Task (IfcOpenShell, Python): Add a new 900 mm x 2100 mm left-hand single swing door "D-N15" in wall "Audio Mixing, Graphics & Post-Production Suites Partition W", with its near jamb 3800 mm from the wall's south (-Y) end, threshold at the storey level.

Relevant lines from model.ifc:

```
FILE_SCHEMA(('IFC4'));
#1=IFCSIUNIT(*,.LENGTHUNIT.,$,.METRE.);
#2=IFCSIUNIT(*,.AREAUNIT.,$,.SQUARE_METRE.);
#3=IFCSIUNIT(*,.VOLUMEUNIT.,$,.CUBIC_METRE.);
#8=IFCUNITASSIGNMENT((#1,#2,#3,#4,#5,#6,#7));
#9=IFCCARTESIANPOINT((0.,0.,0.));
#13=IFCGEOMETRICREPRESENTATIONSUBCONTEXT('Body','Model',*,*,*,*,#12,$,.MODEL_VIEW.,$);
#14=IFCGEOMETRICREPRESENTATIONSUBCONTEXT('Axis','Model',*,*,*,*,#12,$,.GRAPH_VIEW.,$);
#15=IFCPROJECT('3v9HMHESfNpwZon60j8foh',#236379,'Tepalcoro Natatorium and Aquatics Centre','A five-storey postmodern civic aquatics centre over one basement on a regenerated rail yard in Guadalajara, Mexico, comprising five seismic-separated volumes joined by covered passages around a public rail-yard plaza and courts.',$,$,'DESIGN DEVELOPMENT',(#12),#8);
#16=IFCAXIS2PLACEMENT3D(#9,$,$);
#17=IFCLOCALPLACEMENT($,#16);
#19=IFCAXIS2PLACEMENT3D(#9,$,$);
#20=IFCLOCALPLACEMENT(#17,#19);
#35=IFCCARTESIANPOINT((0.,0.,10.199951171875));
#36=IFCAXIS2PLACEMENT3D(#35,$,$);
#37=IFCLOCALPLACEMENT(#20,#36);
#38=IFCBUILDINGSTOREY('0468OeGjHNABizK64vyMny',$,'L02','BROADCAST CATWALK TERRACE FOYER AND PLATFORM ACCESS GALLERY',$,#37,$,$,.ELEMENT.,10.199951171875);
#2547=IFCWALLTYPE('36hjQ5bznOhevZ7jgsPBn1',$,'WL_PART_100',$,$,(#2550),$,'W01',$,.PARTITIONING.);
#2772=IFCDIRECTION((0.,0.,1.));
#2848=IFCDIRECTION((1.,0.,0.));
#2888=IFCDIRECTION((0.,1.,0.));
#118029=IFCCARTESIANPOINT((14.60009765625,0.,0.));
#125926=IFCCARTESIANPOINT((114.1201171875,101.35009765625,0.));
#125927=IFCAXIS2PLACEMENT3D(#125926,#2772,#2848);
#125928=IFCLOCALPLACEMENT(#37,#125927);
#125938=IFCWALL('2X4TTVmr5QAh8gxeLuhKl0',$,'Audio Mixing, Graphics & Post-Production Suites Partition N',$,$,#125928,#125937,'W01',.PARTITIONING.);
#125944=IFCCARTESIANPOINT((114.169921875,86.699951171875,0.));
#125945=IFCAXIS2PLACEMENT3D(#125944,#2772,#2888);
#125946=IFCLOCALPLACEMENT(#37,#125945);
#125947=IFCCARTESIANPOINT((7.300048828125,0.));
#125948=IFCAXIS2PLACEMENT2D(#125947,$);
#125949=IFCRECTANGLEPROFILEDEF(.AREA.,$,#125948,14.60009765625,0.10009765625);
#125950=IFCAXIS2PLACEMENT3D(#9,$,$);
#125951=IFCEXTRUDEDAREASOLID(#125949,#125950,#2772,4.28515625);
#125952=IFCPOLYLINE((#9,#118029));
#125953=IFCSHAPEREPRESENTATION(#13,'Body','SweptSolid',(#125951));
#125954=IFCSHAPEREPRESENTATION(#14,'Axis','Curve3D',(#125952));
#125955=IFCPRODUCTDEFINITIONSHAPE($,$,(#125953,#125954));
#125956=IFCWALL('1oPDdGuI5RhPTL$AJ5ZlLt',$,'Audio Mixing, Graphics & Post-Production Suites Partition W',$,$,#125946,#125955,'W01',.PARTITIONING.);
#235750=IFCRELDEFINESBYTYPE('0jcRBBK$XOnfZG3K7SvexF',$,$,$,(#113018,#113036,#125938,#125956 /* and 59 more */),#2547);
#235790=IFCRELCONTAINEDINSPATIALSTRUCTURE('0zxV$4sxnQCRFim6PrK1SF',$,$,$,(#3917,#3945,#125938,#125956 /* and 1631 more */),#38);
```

```python
import numpy as np
import ifcopenshell
import ifcopenshell.api.feature
import ifcopenshell.api.geometry
import ifcopenshell.api.root
import ifcopenshell.api.spatial
import ifcopenshell.geom
import ifcopenshell.util.element
import ifcopenshell.util.placement
import ifcopenshell.util.representation
import ifcopenshell.util.shape
import ifcopenshell.util.unit

model = ifcopenshell.open("model.ifc")
unit_scale = ifcopenshell.util.unit.calculate_unit_scale(model)
settings = ifcopenshell.geom.settings()


def volume(element):
    """Net volume in cubic metres, openings subtracted."""
    shape = ifcopenshell.geom.create_shape(settings, element)
    return ifcopenshell.util.shape.get_volume(shape.geometry)


wall = model.by_guid("1oPDdGuI5RhPTL$AJ5ZlLt")
storey = ifcopenshell.util.element.get_container(wall, ifc_class="IfcBuildingStorey")
context = ifcopenshell.util.representation.get_context(model, "Model", "Body", "MODEL_VIEW")
before = volume(wall)

width, height, from_end, sill = 0.9, 2.1, 3.8, 0.0  # metres

# The wall runs along its own X axis, and the end named is its -X end.
wall_shape = ifcopenshell.geom.create_shape(settings, wall)
x, y, z = ifcopenshell.util.shape.get_vertices(wall_shape.geometry).T
start = x.min() + from_end
face, thickness = float(y.min()), float(y.max() - y.min())
wall_matrix = ifcopenshell.util.placement.get_local_placement(wall.ObjectPlacement)
level = ifcopenshell.util.placement.get_local_placement(storey.ObjectPlacement)[2, 3]


def in_wall(x, y):
    """Placement at x, y metres in the wall's axes, at sill height."""
    matrix = wall_matrix.copy()
    matrix[:, 3] = wall_matrix @ np.array([x / unit_scale, y / unit_scale, 0.0, 1.0])
    matrix[2, 3] = level + sill / unit_scale
    return matrix


# Opening: a box that overshoots both wall faces by 50 mm.
opening = ifcopenshell.api.root.create_entity(model, ifc_class="IfcOpeningElement", predefined_type="OPENING")
box = ifcopenshell.api.geometry.add_wall_representation(
    model, context=context, length=width, height=height, thickness=thickness + 0.1
)
ifcopenshell.api.geometry.assign_representation(model, product=opening, representation=box)
ifcopenshell.api.geometry.edit_object_placement(model, product=opening, matrix=in_wall(start, face - 0.05), is_si=False)
ifcopenshell.api.feature.add_feature(model, feature=opening, element=wall)

door = ifcopenshell.api.root.create_entity(model, ifc_class="IfcDoor", name="D-N15", predefined_type="DOOR")
door.OverallWidth, door.OverallHeight = width / unit_scale, height / unit_scale
door.OperationType = "SINGLE_SWING_LEFT"
body = ifcopenshell.api.geometry.add_door_representation(
    model,
    context=context,
    overall_width=door.OverallWidth,
    overall_height=door.OverallHeight,
    operation_type="SINGLE_SWING_LEFT",
    lining_properties={"LiningDepth": thickness / unit_scale, "ThresholdDepth": thickness / unit_scale},
)
ifcopenshell.api.geometry.assign_representation(model, product=door, representation=body)
ifcopenshell.api.spatial.assign_container(model, products=[door], relating_structure=storey)
ifcopenshell.api.feature.add_filling(model, opening=opening, element=door)

# The lining spans the wall, so the door starts at the wall face.
ifcopenshell.api.geometry.edit_object_placement(model, product=door, matrix=in_wall(start, face), is_si=False)

after = volume(wall)

print(f"wall volume {before:.3f} -> {after:.3f} m3")

model.write("model-out.ifc")
```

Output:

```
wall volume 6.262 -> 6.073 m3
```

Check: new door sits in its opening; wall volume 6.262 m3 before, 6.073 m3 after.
